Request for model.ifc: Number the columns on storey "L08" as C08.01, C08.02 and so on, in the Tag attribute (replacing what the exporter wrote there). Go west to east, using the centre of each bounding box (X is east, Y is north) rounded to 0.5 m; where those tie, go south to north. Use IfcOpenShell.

First a look at what the model holds.

```python
import ifcopenshell
import ifcopenshell.util.element
import ifcopenshell.util.placement

model = ifcopenshell.open("model.ifc")
print(model.schema)
storey = next(s for s in model.by_type("IfcBuildingStorey") if s.Name == "L08")
columns = [e for e in ifcopenshell.util.element.get_decomposition(storey) if e.is_a("IfcColumn")]
for e in sorted(columns, key=lambda e: e.id()):
    origin = ifcopenshell.util.placement.get_local_placement(e.ObjectPlacement)[:3, 3]
    print(e.id(), e.Tag, e.Name, origin.round(2) + 0.0, sep=" | ")
```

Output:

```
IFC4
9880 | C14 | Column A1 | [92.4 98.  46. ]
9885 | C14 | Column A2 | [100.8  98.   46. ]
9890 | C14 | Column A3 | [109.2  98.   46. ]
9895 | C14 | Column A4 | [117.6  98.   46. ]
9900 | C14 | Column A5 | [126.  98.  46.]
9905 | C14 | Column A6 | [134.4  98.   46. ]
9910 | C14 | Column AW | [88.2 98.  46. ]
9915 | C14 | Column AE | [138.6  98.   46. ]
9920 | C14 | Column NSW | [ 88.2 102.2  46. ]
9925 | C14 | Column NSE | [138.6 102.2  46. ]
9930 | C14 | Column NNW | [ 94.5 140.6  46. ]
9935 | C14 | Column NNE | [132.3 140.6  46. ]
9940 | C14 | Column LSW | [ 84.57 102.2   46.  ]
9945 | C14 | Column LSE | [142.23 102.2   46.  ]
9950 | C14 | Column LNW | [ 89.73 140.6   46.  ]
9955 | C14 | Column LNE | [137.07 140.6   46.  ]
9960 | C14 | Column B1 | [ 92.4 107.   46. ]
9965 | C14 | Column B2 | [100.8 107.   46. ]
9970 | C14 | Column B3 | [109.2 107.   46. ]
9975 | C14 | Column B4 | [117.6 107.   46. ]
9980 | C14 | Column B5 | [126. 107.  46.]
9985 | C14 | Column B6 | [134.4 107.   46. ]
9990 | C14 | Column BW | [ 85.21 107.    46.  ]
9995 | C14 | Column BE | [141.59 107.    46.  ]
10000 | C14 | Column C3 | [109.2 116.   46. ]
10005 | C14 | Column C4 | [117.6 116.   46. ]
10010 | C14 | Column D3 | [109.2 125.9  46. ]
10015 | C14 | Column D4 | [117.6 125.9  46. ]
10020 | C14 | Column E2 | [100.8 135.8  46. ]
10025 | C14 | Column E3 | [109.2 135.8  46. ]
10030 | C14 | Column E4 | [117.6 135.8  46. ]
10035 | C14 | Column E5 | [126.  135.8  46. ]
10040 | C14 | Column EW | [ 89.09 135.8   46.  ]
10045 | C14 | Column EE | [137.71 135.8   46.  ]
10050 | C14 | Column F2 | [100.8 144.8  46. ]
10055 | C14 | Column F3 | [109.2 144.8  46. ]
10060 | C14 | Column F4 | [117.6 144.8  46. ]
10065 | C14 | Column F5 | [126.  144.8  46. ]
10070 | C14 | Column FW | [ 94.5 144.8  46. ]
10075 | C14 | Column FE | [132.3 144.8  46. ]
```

```python
import ifcopenshell
import ifcopenshell.geom
import ifcopenshell.util.element
import ifcopenshell.util.shape

model = ifcopenshell.open("model.ifc")
settings = ifcopenshell.geom.settings()
settings.set("use-world-coords", True)


def centre(element):
    shape = ifcopenshell.geom.create_shape(settings, element)
    return ifcopenshell.util.shape.get_bbox_centroid(shape.geometry)


storey = next(s for s in model.by_type("IfcBuildingStorey") if s.Name == "L08")
columns = [e for e in ifcopenshell.util.element.get_decomposition(storey) if e.is_a("IfcColumn")]

# Insertion points can sit at a corner or the storey origin, so sort by the geometry (in metres).
centres = {e: centre(e) for e in columns}
columns.sort(key=lambda e: (round(centres[e][0] / 0.5), centres[e][1]))

for i, e in enumerate(columns, start=1):
    number = f"C08.{i:02d}"
    e.Tag = number
    print(e.id(), number)

model.write("model-out.ifc")
```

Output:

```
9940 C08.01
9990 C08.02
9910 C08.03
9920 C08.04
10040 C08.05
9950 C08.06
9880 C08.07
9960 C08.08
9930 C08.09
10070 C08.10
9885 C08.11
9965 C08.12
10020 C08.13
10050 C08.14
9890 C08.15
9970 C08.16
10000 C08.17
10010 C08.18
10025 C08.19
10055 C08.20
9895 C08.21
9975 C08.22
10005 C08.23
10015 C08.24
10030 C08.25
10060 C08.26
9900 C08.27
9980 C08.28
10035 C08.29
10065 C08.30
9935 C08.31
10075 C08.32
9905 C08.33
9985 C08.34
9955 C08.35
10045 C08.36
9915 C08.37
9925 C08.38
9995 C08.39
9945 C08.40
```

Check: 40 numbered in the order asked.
